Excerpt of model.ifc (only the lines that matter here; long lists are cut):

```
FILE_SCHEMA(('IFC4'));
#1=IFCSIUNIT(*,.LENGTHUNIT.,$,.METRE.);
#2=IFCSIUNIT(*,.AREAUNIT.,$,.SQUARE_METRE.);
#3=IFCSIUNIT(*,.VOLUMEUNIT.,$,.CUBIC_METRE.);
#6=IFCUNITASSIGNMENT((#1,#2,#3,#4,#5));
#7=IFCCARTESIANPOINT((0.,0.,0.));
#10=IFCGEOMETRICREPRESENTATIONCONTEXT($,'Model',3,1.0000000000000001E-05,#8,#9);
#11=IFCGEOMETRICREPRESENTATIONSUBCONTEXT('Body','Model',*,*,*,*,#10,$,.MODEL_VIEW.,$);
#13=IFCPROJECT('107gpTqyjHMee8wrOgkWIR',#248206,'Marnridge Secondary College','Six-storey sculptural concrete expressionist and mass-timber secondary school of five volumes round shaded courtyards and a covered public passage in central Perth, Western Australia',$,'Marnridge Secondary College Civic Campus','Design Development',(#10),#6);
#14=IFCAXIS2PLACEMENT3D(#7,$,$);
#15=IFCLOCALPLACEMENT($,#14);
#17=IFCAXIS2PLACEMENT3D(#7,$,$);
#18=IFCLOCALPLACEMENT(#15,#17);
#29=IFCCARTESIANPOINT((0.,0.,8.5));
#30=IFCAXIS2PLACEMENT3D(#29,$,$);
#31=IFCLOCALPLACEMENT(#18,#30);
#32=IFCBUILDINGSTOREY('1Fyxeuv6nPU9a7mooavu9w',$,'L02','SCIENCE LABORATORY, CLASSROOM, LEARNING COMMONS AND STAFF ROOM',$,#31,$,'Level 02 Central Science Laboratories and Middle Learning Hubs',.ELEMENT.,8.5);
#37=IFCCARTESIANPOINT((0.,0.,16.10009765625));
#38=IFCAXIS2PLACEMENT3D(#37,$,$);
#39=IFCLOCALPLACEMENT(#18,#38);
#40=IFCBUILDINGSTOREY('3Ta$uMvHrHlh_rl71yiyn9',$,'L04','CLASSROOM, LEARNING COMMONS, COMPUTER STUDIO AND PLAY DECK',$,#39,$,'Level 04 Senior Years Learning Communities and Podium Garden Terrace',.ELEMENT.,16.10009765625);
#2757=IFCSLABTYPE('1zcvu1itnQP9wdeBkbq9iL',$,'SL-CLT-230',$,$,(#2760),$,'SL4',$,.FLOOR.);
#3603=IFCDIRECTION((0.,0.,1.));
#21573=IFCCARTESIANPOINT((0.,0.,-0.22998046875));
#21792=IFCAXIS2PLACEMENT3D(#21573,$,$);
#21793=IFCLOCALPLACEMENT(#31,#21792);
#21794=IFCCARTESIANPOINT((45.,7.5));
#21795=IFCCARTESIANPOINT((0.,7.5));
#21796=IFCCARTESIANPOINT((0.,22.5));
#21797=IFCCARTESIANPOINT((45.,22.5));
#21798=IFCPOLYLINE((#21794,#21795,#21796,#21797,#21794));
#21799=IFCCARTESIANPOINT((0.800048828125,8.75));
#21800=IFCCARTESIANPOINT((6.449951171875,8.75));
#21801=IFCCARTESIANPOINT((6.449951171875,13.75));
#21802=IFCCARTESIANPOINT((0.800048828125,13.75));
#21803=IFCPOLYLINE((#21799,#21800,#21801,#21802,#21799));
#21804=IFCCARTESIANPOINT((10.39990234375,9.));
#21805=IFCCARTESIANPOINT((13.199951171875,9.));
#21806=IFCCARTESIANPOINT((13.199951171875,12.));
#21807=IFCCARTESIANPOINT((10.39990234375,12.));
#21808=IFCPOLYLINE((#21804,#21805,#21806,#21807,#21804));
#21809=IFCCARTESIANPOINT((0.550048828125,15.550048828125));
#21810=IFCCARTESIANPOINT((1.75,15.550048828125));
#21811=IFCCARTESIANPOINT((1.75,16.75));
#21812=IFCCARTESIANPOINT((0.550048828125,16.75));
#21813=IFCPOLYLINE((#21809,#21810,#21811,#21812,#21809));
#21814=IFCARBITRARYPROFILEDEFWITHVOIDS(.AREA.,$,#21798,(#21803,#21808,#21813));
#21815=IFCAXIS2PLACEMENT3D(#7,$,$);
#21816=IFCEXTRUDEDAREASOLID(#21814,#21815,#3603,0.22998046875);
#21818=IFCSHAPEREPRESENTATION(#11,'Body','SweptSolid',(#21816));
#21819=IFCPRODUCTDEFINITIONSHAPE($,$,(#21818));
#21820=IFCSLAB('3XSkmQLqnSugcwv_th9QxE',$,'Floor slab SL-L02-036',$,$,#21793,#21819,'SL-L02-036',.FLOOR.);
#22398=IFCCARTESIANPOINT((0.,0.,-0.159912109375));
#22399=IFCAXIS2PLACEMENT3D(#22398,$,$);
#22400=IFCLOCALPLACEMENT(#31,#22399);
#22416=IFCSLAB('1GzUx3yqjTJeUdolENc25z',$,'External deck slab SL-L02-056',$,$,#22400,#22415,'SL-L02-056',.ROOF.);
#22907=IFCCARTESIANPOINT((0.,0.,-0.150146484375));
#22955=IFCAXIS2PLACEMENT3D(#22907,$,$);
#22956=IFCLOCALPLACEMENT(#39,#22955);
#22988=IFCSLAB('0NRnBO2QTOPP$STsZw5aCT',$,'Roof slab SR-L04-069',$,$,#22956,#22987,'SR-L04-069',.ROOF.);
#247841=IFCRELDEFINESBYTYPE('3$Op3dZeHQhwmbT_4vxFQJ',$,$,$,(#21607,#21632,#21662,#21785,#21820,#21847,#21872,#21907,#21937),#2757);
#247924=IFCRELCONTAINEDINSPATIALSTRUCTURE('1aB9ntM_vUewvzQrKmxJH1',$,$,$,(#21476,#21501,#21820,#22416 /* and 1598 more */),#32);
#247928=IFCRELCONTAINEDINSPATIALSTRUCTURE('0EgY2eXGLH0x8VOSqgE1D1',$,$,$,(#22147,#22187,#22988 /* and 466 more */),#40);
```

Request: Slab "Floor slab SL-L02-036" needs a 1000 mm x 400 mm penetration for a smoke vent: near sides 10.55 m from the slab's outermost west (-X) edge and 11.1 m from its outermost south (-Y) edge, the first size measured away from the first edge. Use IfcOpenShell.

```python
import numpy as np
import ifcopenshell
import ifcopenshell.api.feature
import ifcopenshell.api.geometry
import ifcopenshell.api.root
import ifcopenshell.geom
import ifcopenshell.util.placement
import ifcopenshell.util.representation
import ifcopenshell.util.shape
import ifcopenshell.util.unit

model = ifcopenshell.open("model.ifc")
unit_scale = ifcopenshell.util.unit.calculate_unit_scale(model)
settings = ifcopenshell.geom.settings()


def volume(element):
    """Net volume in cubic metres, openings subtracted."""
    shape = ifcopenshell.geom.create_shape(settings, element)
    return ifcopenshell.util.shape.get_volume(shape.geometry)


slab = model.by_guid("3XSkmQLqnSugcwv_th9QxE")
before = volume(slab)

# Extent in the slab's own axes, in metres. The edges named are its -X and -Y sides.
slab_shape = ifcopenshell.geom.create_shape(settings, slab)
vertices = ifcopenshell.util.shape.get_vertices(slab_shape.geometry)
x_min, y_min, bottom = vertices.min(axis=0)
top = vertices[:, 2].max()

opening = ifcopenshell.api.root.create_entity(model, ifc_class="IfcOpeningElement", name="Smoke vent opening", predefined_type="OPENING")
context = ifcopenshell.util.representation.get_context(model, "Model", "Body", "MODEL_VIEW")
width, depth = 1, 0.4
outline = [(0.0, 0.0), (width, 0.0), (width, depth), (0.0, depth), (0.0, 0.0)]
# Overshoot both faces by 50 mm so the cut is clean.
shape = ifcopenshell.api.geometry.add_slab_representation(
    model, context=context, depth=top - bottom + 0.1, polyline=outline
)
ifcopenshell.api.geometry.assign_representation(model, product=opening, representation=shape)

matrix = ifcopenshell.util.placement.get_local_placement(slab.ObjectPlacement)
matrix[:, 3] = matrix @ np.append(np.array([x_min + 10.55, y_min + 11.1, bottom - 0.05]) / unit_scale, 1.0)
ifcopenshell.api.geometry.edit_object_placement(model, product=opening, matrix=matrix, is_si=False)
ifcopenshell.api.feature.add_feature(model, feature=opening, element=slab)

after = volume(slab)

print(f"slab volume {before:.3f} -> {after:.3f} m3")

model.write("model-out.ifc")
```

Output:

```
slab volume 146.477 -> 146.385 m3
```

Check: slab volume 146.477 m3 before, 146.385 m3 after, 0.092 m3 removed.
